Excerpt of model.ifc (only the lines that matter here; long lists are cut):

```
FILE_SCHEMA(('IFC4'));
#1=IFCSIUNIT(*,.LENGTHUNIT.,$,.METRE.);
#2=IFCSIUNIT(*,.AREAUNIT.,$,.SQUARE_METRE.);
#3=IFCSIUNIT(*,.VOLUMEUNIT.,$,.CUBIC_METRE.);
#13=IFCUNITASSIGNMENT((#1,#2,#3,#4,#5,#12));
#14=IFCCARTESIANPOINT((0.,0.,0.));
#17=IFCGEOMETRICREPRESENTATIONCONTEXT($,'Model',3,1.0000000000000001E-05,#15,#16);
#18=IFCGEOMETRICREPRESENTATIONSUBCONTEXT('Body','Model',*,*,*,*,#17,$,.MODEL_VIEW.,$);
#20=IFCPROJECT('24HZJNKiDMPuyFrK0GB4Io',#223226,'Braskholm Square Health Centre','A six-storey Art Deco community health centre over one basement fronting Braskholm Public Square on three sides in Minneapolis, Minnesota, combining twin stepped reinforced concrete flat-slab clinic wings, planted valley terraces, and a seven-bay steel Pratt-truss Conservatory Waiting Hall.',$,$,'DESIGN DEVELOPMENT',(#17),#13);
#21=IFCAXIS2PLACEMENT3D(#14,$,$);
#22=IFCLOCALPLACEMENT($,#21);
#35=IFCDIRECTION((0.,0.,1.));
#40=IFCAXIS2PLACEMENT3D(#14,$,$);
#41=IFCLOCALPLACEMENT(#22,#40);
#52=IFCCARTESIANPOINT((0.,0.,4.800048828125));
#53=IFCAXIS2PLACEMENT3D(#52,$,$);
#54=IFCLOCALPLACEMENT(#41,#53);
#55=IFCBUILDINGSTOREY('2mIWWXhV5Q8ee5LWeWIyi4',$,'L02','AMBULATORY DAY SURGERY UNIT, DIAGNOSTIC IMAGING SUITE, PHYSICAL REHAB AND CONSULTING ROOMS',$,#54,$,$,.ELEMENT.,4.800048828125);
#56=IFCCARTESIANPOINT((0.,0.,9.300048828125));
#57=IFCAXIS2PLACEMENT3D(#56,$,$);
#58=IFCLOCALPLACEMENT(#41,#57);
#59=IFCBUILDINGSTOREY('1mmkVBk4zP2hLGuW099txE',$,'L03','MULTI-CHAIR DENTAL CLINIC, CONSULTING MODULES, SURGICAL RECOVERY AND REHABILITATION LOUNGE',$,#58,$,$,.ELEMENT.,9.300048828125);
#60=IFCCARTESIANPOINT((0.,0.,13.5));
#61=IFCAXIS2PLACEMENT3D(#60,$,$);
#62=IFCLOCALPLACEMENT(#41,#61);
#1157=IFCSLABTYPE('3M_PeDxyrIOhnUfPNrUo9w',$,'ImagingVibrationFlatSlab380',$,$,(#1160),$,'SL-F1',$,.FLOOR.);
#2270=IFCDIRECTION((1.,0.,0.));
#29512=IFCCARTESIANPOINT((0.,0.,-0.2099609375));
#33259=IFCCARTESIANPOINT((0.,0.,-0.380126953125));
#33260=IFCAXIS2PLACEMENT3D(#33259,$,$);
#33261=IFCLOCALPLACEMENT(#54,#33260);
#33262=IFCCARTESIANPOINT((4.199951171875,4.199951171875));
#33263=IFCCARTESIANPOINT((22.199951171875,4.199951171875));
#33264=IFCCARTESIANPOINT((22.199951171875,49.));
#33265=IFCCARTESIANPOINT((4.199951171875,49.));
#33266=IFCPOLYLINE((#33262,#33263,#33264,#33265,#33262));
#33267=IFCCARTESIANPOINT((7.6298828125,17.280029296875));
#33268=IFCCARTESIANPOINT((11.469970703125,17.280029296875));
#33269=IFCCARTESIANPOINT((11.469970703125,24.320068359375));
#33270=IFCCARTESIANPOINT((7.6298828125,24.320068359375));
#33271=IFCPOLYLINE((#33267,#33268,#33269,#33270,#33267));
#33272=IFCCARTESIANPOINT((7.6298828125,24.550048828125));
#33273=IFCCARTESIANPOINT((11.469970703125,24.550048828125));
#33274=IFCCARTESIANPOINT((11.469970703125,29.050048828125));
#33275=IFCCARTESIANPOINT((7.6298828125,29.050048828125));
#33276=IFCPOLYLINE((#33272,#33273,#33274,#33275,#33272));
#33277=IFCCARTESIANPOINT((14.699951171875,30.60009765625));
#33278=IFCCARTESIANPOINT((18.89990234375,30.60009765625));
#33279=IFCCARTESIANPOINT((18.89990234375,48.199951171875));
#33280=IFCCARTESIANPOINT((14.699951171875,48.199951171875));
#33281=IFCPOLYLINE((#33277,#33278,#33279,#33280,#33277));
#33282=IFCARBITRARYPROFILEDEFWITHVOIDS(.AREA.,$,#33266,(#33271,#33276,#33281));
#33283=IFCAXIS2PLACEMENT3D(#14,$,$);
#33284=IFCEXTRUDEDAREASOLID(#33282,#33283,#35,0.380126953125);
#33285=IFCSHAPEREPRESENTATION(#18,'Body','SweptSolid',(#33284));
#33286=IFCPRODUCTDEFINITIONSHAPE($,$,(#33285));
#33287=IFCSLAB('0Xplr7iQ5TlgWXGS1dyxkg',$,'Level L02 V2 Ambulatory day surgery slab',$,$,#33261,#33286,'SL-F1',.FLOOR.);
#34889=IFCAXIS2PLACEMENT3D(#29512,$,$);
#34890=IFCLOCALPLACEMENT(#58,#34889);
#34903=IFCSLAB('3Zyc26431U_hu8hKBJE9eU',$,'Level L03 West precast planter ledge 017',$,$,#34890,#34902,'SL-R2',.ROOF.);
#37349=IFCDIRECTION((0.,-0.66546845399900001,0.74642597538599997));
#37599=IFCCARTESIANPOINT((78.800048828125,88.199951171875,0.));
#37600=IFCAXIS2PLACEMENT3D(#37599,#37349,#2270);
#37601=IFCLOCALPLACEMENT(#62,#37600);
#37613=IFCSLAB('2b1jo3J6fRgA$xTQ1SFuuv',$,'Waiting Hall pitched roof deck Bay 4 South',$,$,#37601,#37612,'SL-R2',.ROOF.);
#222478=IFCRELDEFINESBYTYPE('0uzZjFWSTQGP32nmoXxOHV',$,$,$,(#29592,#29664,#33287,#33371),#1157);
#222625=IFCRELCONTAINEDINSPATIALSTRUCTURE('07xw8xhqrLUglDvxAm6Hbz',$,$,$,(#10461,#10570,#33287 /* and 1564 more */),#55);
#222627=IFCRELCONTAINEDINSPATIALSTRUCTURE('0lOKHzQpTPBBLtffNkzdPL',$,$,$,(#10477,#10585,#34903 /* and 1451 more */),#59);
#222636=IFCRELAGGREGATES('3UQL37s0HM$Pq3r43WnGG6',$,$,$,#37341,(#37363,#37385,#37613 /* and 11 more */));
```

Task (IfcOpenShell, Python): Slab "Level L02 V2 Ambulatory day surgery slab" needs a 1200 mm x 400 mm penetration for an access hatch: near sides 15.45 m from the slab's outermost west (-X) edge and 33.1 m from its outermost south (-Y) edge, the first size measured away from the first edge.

```python
import numpy as np
import ifcopenshell
import ifcopenshell.api.feature
import ifcopenshell.api.geometry
import ifcopenshell.api.root
import ifcopenshell.geom
import ifcopenshell.util.placement
import ifcopenshell.util.representation
import ifcopenshell.util.shape
import ifcopenshell.util.unit

model = ifcopenshell.open("model.ifc")
unit_scale = ifcopenshell.util.unit.calculate_unit_scale(model)
settings = ifcopenshell.geom.settings()


def volume(element):
    """Net volume in cubic metres, openings subtracted."""
    shape = ifcopenshell.geom.create_shape(settings, element)
    return ifcopenshell.util.shape.get_volume(shape.geometry)


slab = model.by_id(33287)
before = volume(slab)

# Extent in the slab's own axes, in metres. The edges named are its -X and -Y sides.
slab_shape = ifcopenshell.geom.create_shape(settings, slab)
vertices = ifcopenshell.util.shape.get_vertices(slab_shape.geometry)
x_min, y_min, bottom = vertices.min(axis=0)
top = vertices[:, 2].max()

opening = ifcopenshell.api.root.create_entity(model, ifc_class="IfcOpeningElement", name="Access hatch opening", predefined_type="OPENING")
context = ifcopenshell.util.representation.get_context(model, "Model", "Body", "MODEL_VIEW")
width, depth = 1.2, 0.4
outline = [(0.0, 0.0), (width, 0.0), (width, depth), (0.0, depth), (0.0, 0.0)]
# Overshoot both faces by 50 mm so the cut is clean.
shape = ifcopenshell.api.geometry.add_slab_representation(
    model, context=context, depth=top - bottom + 0.1, polyline=outline
)
ifcopenshell.api.geometry.assign_representation(model, product=opening, representation=shape)

matrix = ifcopenshell.util.placement.get_local_placement(slab.ObjectPlacement)
matrix[:, 3] = matrix @ np.append(np.array([x_min + 15.45, y_min + 33.1, bottom - 0.05]) / unit_scale, 1.0)
ifcopenshell.api.geometry.edit_object_placement(model, product=opening, matrix=matrix, is_si=False)
ifcopenshell.api.feature.add_feature(model, feature=opening, element=slab)

after = volume(slab)

print(f"slab volume {before:.3f} -> {after:.3f} m3")

model.write("model_rev.ifc")
```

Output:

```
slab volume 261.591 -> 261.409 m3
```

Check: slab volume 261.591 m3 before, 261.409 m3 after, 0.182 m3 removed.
